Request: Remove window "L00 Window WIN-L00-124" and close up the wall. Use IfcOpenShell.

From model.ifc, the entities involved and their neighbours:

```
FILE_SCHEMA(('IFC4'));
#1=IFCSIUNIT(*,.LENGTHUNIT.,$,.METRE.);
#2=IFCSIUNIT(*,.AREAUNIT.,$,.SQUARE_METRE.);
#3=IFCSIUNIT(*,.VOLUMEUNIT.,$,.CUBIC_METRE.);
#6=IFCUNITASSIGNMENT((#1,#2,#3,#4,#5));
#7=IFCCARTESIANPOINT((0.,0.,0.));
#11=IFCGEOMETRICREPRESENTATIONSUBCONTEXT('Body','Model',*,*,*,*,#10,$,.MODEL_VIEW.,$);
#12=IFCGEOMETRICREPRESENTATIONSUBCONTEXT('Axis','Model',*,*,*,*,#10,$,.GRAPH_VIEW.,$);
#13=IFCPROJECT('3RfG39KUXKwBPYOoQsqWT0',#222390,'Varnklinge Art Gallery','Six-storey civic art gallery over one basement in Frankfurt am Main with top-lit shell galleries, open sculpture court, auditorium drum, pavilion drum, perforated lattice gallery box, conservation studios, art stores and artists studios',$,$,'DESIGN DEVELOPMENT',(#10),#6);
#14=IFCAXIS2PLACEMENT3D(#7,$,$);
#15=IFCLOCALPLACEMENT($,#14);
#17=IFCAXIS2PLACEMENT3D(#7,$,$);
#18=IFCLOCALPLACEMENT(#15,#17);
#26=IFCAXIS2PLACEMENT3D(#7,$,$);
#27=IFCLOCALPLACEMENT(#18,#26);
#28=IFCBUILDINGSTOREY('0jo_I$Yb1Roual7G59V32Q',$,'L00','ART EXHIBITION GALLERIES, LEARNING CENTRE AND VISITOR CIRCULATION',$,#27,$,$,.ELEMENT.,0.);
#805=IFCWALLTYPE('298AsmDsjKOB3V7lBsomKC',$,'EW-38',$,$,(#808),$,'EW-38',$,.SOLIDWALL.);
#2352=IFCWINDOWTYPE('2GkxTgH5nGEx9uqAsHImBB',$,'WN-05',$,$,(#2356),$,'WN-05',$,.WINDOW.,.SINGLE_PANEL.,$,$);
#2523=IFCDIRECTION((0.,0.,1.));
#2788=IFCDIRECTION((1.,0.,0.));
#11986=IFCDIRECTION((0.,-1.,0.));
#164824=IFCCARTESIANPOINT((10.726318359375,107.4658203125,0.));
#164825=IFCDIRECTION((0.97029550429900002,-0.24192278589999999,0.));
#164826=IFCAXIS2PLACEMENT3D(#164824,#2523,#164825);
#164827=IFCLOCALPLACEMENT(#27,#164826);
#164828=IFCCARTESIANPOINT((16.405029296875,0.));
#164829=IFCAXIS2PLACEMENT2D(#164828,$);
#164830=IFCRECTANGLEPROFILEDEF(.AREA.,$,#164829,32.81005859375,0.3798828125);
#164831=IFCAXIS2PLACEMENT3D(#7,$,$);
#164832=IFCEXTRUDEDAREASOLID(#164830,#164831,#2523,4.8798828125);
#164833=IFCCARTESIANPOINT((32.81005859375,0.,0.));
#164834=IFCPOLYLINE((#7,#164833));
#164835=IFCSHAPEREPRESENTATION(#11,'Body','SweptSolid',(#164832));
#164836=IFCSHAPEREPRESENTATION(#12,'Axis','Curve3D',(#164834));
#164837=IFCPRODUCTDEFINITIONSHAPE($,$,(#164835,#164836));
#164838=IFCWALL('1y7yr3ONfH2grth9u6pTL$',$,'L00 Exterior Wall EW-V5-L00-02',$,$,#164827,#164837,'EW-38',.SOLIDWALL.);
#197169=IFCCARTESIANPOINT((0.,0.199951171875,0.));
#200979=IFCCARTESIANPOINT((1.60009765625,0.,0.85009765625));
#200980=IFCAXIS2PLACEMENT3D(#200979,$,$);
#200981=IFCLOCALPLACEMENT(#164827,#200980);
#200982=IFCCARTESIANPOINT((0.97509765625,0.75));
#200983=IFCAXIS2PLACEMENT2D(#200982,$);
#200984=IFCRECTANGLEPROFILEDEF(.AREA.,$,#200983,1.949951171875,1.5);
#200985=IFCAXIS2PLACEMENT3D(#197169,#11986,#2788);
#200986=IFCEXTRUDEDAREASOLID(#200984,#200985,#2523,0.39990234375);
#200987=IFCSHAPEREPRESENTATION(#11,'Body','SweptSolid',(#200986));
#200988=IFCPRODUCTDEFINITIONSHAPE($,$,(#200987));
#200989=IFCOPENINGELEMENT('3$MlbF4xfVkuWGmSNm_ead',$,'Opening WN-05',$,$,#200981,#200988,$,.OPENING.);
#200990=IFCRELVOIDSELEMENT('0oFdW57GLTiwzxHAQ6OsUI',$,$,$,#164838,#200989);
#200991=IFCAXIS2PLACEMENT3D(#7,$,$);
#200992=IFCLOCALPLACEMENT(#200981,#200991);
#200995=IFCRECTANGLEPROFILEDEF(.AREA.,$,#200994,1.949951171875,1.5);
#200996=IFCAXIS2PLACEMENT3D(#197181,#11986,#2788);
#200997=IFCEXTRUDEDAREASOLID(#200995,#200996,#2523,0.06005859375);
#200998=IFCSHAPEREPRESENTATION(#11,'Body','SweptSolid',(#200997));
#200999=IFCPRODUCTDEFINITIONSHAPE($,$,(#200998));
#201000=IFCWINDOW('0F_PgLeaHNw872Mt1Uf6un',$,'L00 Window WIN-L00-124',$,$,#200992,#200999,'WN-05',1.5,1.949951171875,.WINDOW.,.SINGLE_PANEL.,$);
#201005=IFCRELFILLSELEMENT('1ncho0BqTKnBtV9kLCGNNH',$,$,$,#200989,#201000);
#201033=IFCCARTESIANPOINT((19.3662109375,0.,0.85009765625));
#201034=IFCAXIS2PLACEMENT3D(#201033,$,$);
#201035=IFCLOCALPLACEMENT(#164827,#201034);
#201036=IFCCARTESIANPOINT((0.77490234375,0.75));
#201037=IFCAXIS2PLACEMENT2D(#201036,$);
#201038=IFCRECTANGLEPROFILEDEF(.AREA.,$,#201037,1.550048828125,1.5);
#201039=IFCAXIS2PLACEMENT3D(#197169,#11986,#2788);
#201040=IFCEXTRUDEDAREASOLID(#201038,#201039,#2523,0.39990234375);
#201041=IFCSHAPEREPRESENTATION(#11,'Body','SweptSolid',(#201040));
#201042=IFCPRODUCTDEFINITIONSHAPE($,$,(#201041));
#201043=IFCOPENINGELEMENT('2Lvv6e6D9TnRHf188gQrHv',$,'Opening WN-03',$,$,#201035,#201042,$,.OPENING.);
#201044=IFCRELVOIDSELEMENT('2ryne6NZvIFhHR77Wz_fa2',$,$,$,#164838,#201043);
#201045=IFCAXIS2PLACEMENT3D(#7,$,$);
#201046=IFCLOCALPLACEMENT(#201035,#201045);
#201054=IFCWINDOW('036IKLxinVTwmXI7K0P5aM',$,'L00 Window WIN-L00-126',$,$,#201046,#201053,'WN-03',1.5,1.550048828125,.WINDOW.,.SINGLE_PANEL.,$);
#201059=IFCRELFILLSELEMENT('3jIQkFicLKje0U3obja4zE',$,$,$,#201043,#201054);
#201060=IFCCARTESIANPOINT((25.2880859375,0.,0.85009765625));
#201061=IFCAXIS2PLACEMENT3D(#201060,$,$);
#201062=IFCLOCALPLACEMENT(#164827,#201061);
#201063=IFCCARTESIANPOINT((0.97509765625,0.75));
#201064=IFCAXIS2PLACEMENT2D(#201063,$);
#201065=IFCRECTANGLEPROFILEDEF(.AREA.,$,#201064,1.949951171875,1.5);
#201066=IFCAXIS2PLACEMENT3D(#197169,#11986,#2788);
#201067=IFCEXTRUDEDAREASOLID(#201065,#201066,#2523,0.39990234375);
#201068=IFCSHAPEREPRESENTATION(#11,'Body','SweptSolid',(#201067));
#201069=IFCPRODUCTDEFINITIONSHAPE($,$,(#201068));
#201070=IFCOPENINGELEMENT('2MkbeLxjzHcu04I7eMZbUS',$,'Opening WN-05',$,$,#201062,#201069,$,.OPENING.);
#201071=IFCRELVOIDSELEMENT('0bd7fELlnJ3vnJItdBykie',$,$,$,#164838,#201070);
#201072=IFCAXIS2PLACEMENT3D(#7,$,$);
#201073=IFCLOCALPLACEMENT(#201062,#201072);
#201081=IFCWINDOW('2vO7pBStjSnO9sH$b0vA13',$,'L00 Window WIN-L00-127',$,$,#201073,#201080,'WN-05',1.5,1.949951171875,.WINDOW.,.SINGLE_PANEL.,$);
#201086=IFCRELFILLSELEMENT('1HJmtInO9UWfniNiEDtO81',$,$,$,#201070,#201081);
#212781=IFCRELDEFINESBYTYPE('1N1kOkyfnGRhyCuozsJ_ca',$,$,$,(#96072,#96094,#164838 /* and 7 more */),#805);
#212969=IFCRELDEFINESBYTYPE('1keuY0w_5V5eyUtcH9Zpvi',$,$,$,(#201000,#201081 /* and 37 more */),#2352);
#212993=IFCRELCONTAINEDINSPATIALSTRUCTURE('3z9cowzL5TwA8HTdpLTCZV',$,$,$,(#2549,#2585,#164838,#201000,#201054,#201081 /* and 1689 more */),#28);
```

```python
import ifcopenshell
import ifcopenshell.api.feature
import ifcopenshell.api.root
import ifcopenshell.geom
import ifcopenshell.util.shape

model = ifcopenshell.open("model.ifc")
settings = ifcopenshell.geom.settings()


def volume(element):
    """Net volume in cubic metres, openings subtracted."""
    shape = ifcopenshell.geom.create_shape(settings, element)
    return ifcopenshell.util.shape.get_volume(shape.geometry)


window = model.by_id(201000)
opening = window.FillsVoids[0].RelatingOpeningElement
wall = opening.VoidsElements[0].RelatingBuildingElement
before = volume(wall)

ifcopenshell.api.root.remove_product(model, product=window)
ifcopenshell.api.feature.remove_feature(model, feature=opening)

after = volume(wall)

print(f"wall volume {before:.3f} -> {after:.3f} m3")

model.write("model_edited.ifc")
```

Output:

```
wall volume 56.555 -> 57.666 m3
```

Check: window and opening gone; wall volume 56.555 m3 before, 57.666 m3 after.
